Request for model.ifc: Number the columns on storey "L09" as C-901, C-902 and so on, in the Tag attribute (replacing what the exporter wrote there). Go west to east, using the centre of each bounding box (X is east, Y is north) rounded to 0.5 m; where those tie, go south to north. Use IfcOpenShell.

First a look at what the model holds.

```python
import ifcopenshell
import ifcopenshell.util.element
import ifcopenshell.util.placement

model = ifcopenshell.open("model.ifc")
print(model.schema)
storey = next(s for s in model.by_type("IfcBuildingStorey") if s.Name == "L09")
columns = [e for e in ifcopenshell.util.element.get_decomposition(storey) if e.is_a("IfcColumn")]
for e in sorted(columns, key=lambda e: e.id()):
    origin = ifcopenshell.util.placement.get_local_placement(e.ObjectPlacement)[:3, 3]
    print(e.id(), e.Tag, e.Name, origin.round(2) + 0.0, sep=" | ")
```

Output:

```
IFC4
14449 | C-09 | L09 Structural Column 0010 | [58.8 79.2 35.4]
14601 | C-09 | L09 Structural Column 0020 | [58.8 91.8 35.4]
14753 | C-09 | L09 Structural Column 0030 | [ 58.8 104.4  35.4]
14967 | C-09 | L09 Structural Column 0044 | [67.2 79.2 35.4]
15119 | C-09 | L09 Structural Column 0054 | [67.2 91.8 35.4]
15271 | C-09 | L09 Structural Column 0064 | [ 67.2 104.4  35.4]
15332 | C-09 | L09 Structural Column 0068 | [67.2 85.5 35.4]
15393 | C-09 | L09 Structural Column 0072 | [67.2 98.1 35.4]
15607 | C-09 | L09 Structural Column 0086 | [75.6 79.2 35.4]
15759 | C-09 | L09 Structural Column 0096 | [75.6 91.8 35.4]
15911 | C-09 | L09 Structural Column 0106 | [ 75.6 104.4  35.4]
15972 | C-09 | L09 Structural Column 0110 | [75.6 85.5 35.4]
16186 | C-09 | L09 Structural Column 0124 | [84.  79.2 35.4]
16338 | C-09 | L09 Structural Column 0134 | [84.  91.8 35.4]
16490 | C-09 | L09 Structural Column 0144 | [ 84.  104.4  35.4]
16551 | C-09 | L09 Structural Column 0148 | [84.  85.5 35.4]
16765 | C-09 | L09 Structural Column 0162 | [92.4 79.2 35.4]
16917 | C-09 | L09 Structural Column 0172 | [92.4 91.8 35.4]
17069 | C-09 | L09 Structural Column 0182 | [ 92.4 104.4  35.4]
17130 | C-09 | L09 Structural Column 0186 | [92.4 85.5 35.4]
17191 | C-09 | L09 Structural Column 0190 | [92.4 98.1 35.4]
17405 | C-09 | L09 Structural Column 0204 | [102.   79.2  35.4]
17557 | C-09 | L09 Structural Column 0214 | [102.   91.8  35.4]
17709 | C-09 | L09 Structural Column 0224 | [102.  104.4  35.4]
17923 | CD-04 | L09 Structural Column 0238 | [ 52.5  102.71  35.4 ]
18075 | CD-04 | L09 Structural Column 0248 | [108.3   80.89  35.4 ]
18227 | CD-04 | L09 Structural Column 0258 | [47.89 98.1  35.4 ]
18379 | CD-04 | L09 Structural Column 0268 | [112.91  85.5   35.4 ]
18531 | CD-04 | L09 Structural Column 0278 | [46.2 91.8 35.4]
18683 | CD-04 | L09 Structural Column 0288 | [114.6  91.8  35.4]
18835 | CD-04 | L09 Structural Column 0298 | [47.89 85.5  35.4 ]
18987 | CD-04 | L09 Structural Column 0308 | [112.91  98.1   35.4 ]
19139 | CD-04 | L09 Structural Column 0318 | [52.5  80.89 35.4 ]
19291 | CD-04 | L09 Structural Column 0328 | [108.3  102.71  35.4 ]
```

```python
import ifcopenshell
import ifcopenshell.geom
import ifcopenshell.util.element
import ifcopenshell.util.shape

model = ifcopenshell.open("model.ifc")
settings = ifcopenshell.geom.settings()
settings.set("use-world-coords", True)


def centre(element):
    shape = ifcopenshell.geom.create_shape(settings, element)
    return ifcopenshell.util.shape.get_bbox_centroid(shape.geometry)


storey = next(s for s in model.by_type("IfcBuildingStorey") if s.Name == "L09")
columns = [e for e in ifcopenshell.util.element.get_decomposition(storey) if e.is_a("IfcColumn")]

# Insertion points can sit at a corner or the storey origin, so sort by the geometry (in metres).
centres = {e: centre(e) for e in columns}
columns.sort(key=lambda e: (round(centres[e][0] / 0.5), centres[e][1]))

for i, e in enumerate(columns, start=1):
    number = f"C-9{i:02d}"
    e.Tag = number
    print(e.id(), number)

model.write("model-out.ifc")
```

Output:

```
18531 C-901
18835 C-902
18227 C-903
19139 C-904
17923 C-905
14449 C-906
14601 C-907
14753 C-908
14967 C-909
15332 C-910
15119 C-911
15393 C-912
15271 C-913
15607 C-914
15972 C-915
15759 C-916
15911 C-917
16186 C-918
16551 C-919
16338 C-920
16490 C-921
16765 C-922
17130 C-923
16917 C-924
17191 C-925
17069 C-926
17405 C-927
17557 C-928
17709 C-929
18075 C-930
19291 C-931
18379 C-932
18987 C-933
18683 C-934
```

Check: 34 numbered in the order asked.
